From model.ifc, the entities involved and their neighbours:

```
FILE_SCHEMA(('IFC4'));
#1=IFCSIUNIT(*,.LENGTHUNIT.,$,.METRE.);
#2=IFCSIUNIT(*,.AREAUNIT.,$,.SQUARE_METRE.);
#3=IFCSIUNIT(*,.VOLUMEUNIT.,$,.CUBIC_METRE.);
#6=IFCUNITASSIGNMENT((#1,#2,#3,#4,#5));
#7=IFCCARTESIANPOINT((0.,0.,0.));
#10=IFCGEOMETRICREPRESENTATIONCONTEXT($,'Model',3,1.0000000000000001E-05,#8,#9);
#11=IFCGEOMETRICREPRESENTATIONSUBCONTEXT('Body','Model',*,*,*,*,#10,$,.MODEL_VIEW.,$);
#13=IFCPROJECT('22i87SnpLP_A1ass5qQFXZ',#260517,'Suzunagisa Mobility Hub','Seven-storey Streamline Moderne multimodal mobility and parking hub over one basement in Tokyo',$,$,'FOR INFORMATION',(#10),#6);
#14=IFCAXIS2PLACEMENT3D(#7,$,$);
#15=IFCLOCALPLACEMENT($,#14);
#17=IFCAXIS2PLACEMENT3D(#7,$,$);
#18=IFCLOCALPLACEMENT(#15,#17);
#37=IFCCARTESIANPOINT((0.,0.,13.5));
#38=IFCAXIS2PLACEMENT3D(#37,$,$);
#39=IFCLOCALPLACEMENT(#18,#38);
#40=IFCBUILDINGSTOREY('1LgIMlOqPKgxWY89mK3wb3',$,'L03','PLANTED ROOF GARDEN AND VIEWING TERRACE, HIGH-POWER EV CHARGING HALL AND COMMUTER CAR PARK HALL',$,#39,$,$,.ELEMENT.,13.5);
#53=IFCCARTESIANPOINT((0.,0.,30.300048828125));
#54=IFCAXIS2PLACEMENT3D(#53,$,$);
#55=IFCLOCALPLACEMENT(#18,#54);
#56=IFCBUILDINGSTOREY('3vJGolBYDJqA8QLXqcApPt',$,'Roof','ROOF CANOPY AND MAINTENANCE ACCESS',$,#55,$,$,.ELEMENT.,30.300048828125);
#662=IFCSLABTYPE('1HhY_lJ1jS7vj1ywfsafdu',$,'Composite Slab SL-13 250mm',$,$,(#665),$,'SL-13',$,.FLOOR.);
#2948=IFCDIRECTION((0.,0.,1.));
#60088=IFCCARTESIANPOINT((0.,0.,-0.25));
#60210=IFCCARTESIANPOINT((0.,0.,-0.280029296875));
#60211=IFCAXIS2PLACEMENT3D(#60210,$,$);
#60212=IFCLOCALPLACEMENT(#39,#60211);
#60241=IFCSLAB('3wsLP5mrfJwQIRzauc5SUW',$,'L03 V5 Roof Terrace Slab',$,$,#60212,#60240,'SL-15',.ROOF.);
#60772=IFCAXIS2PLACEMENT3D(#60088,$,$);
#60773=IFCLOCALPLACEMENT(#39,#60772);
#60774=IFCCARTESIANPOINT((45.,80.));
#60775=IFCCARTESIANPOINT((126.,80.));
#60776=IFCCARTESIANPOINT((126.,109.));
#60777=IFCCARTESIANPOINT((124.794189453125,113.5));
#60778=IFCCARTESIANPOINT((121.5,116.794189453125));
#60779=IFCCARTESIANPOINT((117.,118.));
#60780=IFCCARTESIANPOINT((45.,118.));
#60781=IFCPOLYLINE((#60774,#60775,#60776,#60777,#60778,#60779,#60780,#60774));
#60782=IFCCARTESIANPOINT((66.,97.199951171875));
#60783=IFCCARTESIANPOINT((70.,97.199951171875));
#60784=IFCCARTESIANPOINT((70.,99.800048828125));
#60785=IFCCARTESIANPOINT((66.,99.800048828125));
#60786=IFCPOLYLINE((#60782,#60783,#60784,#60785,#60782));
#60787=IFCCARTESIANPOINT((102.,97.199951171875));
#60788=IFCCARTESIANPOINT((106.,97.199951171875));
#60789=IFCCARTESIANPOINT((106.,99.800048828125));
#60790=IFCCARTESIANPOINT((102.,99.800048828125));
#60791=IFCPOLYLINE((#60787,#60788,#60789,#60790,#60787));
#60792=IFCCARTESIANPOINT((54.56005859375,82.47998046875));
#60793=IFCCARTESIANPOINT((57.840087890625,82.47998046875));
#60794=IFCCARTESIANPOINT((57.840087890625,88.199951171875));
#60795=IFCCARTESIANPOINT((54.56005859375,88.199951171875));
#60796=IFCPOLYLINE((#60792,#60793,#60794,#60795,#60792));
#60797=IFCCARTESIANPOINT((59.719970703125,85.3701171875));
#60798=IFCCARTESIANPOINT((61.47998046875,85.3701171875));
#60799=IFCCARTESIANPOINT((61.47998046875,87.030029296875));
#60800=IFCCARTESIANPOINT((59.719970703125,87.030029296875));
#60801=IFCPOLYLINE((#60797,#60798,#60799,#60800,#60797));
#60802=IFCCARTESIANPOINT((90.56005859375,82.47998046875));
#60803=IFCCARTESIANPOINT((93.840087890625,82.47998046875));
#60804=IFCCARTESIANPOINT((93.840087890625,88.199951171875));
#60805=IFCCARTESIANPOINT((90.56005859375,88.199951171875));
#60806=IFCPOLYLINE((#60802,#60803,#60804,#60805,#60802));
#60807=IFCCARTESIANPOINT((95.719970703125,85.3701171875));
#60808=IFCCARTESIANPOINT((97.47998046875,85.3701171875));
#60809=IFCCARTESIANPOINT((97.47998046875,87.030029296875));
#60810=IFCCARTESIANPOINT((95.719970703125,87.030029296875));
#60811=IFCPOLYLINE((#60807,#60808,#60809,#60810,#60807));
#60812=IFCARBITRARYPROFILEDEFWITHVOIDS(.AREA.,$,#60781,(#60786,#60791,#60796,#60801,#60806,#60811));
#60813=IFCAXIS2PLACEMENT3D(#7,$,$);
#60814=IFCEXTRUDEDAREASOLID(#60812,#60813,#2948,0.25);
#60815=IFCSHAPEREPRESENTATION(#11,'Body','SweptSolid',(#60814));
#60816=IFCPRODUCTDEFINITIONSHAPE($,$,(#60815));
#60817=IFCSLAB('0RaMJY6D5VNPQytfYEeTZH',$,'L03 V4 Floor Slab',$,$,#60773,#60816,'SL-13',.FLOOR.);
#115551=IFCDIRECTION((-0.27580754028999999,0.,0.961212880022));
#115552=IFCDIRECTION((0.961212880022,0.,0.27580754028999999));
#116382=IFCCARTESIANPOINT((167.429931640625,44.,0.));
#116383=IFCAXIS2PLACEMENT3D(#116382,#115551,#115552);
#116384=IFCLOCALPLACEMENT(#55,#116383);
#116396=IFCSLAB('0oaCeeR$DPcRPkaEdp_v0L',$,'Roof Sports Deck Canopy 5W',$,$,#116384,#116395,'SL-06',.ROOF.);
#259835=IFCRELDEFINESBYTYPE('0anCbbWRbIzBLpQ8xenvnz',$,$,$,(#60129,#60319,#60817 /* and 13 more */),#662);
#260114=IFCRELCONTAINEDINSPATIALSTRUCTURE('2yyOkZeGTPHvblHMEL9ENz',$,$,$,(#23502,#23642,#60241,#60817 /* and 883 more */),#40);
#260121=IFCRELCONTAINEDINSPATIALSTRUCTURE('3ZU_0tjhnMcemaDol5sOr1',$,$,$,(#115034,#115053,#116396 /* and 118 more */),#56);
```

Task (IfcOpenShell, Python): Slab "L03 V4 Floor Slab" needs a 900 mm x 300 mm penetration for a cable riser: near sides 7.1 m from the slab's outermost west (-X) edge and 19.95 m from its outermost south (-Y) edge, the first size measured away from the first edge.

```python
import numpy as np
import ifcopenshell
import ifcopenshell.api.feature
import ifcopenshell.api.geometry
import ifcopenshell.api.root
import ifcopenshell.geom
import ifcopenshell.util.placement
import ifcopenshell.util.representation
import ifcopenshell.util.shape
import ifcopenshell.util.unit

model = ifcopenshell.open("model.ifc")
unit_scale = ifcopenshell.util.unit.calculate_unit_scale(model)
settings = ifcopenshell.geom.settings()


def volume(element):
    """Net volume in cubic metres, openings subtracted."""
    shape = ifcopenshell.geom.create_shape(settings, element)
    return ifcopenshell.util.shape.get_volume(shape.geometry)


slab = model.by_id(60817)
before = volume(slab)

# Extent in the slab's own axes, in metres. The edges named are its -X and -Y sides.
slab_shape = ifcopenshell.geom.create_shape(settings, slab)
vertices = ifcopenshell.util.shape.get_vertices(slab_shape.geometry)
x_min, y_min, bottom = vertices.min(axis=0)
top = vertices[:, 2].max()

opening = ifcopenshell.api.root.create_entity(model, ifc_class="IfcOpeningElement", name="Cable riser opening", predefined_type="OPENING")
context = ifcopenshell.util.representation.get_context(model, "Model", "Body", "MODEL_VIEW")
width, depth = 0.9, 0.3
outline = [(0.0, 0.0), (width, 0.0), (width, depth), (0.0, depth), (0.0, 0.0)]
# Overshoot both faces by 50 mm so the cut is clean.
shape = ifcopenshell.api.geometry.add_slab_representation(
    model, context=context, depth=top - bottom + 0.1, polyline=outline
)
ifcopenshell.api.geometry.assign_representation(model, product=opening, representation=shape)

matrix = ifcopenshell.util.placement.get_local_placement(slab.ObjectPlacement)
matrix[:, 3] = matrix @ np.append(np.array([x_min + 7.1, y_min + 19.95, bottom - 0.05]) / unit_scale, 1.0)
ifcopenshell.api.geometry.edit_object_placement(model, product=opening, matrix=matrix, is_si=False)
ifcopenshell.api.feature.add_feature(model, feature=opening, element=slab)

after = volume(slab)

print(f"slab volume {before:.3f} -> {after:.3f} m3")

model.write("model_v2.ifc")
```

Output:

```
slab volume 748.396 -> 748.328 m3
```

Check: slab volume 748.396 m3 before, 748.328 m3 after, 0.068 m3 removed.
